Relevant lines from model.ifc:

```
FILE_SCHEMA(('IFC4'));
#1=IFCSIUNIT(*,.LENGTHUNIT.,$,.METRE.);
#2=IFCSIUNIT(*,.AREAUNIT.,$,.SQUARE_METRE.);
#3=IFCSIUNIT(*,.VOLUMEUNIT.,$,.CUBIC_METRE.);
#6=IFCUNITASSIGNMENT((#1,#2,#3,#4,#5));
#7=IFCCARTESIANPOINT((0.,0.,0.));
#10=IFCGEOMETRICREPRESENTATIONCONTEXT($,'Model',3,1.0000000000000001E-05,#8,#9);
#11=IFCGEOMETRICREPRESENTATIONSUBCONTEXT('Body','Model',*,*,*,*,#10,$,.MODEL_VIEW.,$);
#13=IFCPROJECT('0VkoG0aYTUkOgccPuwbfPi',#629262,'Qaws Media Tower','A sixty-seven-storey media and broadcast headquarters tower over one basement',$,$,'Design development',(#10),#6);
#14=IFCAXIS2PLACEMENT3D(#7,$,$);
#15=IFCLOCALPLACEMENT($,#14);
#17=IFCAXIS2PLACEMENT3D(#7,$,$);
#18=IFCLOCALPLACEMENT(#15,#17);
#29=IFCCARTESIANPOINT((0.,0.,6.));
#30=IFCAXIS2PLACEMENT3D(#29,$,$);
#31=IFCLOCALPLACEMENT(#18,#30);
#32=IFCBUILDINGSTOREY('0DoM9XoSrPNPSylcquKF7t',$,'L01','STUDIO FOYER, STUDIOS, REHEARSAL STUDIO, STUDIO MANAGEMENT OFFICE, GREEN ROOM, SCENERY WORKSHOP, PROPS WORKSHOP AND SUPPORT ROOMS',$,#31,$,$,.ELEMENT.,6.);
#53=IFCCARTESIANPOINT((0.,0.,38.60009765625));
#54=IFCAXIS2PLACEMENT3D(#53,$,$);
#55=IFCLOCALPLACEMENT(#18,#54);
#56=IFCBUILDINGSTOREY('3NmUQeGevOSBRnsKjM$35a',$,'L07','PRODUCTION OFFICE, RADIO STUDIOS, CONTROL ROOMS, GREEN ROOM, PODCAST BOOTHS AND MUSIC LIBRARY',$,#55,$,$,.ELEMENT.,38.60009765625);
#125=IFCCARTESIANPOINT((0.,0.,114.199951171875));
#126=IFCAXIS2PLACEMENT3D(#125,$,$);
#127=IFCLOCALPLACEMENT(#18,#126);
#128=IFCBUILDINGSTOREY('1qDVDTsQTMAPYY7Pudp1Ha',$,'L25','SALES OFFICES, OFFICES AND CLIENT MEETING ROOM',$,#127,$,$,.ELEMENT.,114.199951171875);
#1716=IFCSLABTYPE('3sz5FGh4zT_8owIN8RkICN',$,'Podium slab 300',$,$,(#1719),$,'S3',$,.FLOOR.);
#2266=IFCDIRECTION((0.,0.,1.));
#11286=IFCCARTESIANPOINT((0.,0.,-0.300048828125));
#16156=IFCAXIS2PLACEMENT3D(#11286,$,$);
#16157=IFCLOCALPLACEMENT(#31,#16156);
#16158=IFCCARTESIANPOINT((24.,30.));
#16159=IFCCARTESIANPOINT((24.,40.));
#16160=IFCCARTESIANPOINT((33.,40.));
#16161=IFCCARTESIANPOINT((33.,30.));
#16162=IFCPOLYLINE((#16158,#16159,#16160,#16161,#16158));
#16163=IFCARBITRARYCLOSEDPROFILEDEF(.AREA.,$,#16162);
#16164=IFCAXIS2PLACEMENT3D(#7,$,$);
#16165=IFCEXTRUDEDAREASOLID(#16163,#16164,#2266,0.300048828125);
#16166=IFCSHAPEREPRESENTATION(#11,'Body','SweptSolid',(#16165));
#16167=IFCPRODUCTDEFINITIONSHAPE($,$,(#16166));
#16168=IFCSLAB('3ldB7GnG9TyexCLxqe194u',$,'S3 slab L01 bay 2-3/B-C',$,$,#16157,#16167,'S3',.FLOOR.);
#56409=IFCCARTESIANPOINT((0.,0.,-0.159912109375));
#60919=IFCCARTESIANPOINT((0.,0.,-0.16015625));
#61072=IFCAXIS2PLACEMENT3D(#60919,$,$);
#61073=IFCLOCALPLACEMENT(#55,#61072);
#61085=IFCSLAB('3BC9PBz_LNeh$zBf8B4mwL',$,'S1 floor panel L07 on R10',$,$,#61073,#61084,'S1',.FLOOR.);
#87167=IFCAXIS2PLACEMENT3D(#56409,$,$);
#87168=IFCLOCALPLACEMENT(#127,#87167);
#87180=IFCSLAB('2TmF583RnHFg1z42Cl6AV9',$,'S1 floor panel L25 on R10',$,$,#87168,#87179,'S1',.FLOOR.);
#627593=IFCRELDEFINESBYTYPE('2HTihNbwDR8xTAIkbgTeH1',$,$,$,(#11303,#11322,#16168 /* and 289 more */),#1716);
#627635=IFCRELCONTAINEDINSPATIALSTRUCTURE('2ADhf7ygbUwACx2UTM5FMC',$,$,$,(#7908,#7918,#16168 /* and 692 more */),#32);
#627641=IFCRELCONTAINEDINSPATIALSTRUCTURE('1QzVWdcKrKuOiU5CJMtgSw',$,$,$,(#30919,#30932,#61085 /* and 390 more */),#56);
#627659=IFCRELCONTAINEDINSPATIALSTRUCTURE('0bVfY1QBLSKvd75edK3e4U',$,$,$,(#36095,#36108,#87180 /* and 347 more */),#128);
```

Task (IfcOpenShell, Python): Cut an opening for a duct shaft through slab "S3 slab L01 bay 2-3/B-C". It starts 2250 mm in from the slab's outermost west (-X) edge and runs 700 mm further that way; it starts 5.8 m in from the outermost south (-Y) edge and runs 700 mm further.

```python
import numpy as np
import ifcopenshell
import ifcopenshell.api.feature
import ifcopenshell.api.geometry
import ifcopenshell.api.root
import ifcopenshell.geom
import ifcopenshell.util.placement
import ifcopenshell.util.representation
import ifcopenshell.util.shape
import ifcopenshell.util.unit

model = ifcopenshell.open("model.ifc")
unit_scale = ifcopenshell.util.unit.calculate_unit_scale(model)
settings = ifcopenshell.geom.settings()


def volume(element):
    """Net volume in cubic metres, openings subtracted."""
    shape = ifcopenshell.geom.create_shape(settings, element)
    return ifcopenshell.util.shape.get_volume(shape.geometry)


slab = model.by_guid("3ldB7GnG9TyexCLxqe194u")
before = volume(slab)

# Extent in the slab's own axes, in metres. The edges named are its -X and -Y sides.
slab_shape = ifcopenshell.geom.create_shape(settings, slab)
vertices = ifcopenshell.util.shape.get_vertices(slab_shape.geometry)
x_min, y_min, bottom = vertices.min(axis=0)
top = vertices[:, 2].max()

opening = ifcopenshell.api.root.create_entity(model, ifc_class="IfcOpeningElement", name="Duct shaft opening", predefined_type="OPENING")
context = ifcopenshell.util.representation.get_context(model, "Model", "Body", "MODEL_VIEW")
width, depth = 0.7, 0.7
outline = [(0.0, 0.0), (width, 0.0), (width, depth), (0.0, depth), (0.0, 0.0)]
# Overshoot both faces by 50 mm so the cut is clean.
shape = ifcopenshell.api.geometry.add_slab_representation(
    model, context=context, depth=top - bottom + 0.1, polyline=outline
)
ifcopenshell.api.geometry.assign_representation(model, product=opening, representation=shape)

matrix = ifcopenshell.util.placement.get_local_placement(slab.ObjectPlacement)
matrix[:, 3] = matrix @ np.append(np.array([x_min + 2.25, y_min + 5.8, bottom - 0.05]) / unit_scale, 1.0)
ifcopenshell.api.geometry.edit_object_placement(model, product=opening, matrix=matrix, is_si=False)
ifcopenshell.api.feature.add_feature(model, feature=opening, element=slab)

after = volume(slab)

print(f"slab volume {before:.3f} -> {after:.3f} m3")

model.write("model_edited.ifc")
```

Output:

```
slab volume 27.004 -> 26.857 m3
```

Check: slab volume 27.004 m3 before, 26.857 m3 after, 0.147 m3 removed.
